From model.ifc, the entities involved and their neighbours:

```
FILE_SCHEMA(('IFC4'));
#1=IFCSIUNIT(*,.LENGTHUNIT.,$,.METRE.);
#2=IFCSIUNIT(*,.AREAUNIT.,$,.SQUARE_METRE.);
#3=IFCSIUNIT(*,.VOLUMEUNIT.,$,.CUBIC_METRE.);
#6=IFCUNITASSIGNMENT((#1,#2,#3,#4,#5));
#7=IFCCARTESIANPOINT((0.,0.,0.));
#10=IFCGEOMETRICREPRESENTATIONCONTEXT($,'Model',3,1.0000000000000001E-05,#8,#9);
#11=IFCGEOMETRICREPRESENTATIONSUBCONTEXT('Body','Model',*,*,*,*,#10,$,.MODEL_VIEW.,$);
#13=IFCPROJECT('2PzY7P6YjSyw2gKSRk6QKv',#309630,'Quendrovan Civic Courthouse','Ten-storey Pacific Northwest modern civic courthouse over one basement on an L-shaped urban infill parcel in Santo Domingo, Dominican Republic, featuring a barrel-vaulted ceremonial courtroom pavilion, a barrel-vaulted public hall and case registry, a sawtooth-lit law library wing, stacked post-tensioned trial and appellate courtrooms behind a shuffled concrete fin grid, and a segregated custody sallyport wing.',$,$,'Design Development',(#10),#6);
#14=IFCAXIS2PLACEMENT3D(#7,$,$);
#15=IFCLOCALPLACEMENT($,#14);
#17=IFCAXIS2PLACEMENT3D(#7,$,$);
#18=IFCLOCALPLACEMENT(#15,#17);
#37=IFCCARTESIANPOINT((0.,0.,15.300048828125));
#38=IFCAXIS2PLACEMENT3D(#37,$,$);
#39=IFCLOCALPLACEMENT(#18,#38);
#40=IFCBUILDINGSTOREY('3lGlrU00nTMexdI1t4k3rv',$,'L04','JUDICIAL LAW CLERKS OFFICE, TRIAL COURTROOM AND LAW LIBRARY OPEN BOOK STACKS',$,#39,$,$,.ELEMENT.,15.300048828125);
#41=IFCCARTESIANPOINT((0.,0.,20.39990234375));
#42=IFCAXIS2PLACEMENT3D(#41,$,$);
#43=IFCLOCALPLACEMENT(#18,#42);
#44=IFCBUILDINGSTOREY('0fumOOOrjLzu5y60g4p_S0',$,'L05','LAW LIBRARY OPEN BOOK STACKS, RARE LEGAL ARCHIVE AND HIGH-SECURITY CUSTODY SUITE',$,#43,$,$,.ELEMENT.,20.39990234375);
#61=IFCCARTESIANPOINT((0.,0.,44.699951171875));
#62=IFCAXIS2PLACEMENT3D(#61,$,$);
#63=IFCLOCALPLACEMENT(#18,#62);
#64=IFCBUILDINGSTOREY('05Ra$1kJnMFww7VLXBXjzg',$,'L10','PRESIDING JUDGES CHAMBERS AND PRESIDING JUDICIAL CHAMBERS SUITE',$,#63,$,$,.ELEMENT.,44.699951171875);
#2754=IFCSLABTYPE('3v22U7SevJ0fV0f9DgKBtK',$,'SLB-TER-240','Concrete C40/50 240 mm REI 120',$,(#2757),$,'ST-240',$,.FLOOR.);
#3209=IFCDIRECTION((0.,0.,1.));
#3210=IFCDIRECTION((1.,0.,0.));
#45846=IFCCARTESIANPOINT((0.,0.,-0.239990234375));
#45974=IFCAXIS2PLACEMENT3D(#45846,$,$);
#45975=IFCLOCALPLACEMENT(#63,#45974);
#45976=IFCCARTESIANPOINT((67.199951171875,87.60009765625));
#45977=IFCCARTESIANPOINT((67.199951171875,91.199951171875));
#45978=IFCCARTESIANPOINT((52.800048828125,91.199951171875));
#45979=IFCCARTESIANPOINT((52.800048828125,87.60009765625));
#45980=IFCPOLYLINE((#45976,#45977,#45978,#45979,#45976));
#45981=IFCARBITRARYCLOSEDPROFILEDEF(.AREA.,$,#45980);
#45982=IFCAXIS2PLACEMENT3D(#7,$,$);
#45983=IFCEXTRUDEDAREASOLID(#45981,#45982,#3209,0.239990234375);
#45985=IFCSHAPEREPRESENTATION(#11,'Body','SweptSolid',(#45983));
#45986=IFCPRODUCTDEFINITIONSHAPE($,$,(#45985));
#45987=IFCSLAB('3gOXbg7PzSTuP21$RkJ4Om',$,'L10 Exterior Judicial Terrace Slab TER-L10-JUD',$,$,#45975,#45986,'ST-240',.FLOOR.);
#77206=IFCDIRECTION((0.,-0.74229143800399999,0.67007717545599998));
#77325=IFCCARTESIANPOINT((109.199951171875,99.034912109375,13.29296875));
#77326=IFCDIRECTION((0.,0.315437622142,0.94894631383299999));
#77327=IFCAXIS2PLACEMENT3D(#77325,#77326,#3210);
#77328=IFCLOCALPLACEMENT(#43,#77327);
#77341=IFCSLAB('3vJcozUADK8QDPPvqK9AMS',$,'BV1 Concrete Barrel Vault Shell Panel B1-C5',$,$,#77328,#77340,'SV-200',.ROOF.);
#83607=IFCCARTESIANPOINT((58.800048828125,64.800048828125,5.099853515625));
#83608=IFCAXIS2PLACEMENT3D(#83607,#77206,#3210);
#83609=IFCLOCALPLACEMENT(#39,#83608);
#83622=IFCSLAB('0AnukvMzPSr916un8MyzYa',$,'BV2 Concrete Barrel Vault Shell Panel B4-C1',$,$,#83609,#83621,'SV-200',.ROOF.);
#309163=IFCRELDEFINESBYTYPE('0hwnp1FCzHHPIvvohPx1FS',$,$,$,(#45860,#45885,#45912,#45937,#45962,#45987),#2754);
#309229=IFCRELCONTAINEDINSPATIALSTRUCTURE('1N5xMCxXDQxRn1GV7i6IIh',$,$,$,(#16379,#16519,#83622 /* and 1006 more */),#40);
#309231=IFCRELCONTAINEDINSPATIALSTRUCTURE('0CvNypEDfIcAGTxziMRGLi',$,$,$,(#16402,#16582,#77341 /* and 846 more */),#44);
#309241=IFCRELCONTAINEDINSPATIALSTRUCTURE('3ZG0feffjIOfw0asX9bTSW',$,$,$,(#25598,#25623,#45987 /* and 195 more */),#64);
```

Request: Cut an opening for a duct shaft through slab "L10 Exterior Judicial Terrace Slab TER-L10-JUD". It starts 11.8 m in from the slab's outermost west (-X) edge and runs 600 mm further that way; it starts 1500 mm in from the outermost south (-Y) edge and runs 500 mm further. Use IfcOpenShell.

```python
import numpy as np
import ifcopenshell
import ifcopenshell.api.feature
import ifcopenshell.api.geometry
import ifcopenshell.api.root
import ifcopenshell.geom
import ifcopenshell.util.placement
import ifcopenshell.util.representation
import ifcopenshell.util.shape
import ifcopenshell.util.unit

model = ifcopenshell.open("model.ifc")
unit_scale = ifcopenshell.util.unit.calculate_unit_scale(model)
settings = ifcopenshell.geom.settings()


def volume(element):
    """Net volume in cubic metres, openings subtracted."""
    shape = ifcopenshell.geom.create_shape(settings, element)
    return ifcopenshell.util.shape.get_volume(shape.geometry)


slab = model.by_guid("3gOXbg7PzSTuP21$RkJ4Om")
before = volume(slab)

# Extent in the slab's own axes, in metres. The edges named are its -X and -Y sides.
slab_shape = ifcopenshell.geom.create_shape(settings, slab)
vertices = ifcopenshell.util.shape.get_vertices(slab_shape.geometry)
x_min, y_min, bottom = vertices.min(axis=0)
top = vertices[:, 2].max()

opening = ifcopenshell.api.root.create_entity(model, ifc_class="IfcOpeningElement", name="Duct shaft opening", predefined_type="OPENING")
context = ifcopenshell.util.representation.get_context(model, "Model", "Body", "MODEL_VIEW")
width, depth = 0.6, 0.5
outline = [(0.0, 0.0), (width, 0.0), (width, depth), (0.0, depth), (0.0, 0.0)]
# Overshoot both faces by 50 mm so the cut is clean.
shape = ifcopenshell.api.geometry.add_slab_representation(
    model, context=context, depth=top - bottom + 0.1, polyline=outline
)
ifcopenshell.api.geometry.assign_representation(model, product=opening, representation=shape)

matrix = ifcopenshell.util.placement.get_local_placement(slab.ObjectPlacement)
matrix[:, 3] = matrix @ np.append(np.array([x_min + 11.8, y_min + 1.5, bottom - 0.05]) / unit_scale, 1.0)
ifcopenshell.api.geometry.edit_object_placement(model, product=opening, matrix=matrix, is_si=False)
ifcopenshell.api.feature.add_feature(model, feature=opening, element=slab)

after = volume(slab)

print(f"slab volume {before:.3f} -> {after:.3f} m3")

model.write("model-out.ifc")
```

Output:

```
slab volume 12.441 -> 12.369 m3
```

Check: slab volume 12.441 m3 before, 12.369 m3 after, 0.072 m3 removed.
